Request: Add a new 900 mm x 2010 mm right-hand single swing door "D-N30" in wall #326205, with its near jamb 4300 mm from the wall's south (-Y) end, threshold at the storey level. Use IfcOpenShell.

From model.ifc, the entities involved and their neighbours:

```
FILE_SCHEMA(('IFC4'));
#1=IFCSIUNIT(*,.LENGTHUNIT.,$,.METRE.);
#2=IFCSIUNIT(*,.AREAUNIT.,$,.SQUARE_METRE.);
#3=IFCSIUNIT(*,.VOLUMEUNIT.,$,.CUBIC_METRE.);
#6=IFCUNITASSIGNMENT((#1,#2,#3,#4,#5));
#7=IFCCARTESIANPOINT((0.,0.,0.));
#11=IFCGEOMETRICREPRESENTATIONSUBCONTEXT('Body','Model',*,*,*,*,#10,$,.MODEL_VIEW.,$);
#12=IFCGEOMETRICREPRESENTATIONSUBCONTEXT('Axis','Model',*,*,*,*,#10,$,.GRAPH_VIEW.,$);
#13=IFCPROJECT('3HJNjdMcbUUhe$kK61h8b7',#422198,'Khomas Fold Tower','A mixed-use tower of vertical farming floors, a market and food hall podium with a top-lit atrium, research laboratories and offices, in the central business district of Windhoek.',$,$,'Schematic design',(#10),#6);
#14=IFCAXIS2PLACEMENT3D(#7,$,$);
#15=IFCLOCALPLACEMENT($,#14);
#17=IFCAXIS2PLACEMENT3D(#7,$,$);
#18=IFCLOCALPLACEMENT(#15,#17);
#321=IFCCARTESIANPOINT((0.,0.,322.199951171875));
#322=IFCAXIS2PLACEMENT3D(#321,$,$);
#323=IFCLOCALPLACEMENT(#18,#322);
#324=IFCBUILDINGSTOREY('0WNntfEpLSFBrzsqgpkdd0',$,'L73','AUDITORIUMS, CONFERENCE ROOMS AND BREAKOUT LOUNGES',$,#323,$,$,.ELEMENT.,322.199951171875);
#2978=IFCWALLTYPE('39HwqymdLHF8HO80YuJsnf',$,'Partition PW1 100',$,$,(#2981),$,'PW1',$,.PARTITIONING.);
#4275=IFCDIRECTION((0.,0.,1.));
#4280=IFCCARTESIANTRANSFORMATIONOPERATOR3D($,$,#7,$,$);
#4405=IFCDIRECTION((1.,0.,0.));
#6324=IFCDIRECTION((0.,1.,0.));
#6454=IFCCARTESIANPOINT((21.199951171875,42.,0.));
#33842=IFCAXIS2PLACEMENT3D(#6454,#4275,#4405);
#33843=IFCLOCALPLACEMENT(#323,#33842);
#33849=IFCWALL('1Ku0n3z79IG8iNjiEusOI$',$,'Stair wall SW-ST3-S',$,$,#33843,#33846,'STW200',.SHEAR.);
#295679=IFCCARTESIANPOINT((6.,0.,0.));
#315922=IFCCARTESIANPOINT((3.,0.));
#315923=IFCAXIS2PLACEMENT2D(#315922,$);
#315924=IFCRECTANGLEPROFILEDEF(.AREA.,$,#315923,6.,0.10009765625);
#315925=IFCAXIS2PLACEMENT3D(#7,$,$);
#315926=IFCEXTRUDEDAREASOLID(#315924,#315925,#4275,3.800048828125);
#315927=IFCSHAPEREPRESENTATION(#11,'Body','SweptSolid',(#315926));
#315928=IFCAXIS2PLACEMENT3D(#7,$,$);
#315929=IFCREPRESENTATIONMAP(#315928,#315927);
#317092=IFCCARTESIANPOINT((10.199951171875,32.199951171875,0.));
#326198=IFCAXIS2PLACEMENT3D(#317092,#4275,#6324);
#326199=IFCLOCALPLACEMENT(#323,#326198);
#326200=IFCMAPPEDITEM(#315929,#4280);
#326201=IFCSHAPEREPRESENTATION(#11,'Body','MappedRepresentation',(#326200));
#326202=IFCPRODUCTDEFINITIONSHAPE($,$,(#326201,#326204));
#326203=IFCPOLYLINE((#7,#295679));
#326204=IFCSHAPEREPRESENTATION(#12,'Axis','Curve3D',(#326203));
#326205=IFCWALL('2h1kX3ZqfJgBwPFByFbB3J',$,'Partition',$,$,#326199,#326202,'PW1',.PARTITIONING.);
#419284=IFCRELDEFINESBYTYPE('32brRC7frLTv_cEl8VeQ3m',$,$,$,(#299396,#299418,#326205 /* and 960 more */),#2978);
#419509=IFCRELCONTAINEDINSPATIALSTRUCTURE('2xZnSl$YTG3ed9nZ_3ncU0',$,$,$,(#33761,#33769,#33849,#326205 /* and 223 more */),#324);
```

```python
import numpy as np
import ifcopenshell
import ifcopenshell.api.feature
import ifcopenshell.api.geometry
import ifcopenshell.api.root
import ifcopenshell.api.spatial
import ifcopenshell.geom
import ifcopenshell.util.element
import ifcopenshell.util.placement
import ifcopenshell.util.representation
import ifcopenshell.util.shape
import ifcopenshell.util.unit

model = ifcopenshell.open("model.ifc")
unit_scale = ifcopenshell.util.unit.calculate_unit_scale(model)
settings = ifcopenshell.geom.settings()


def volume(element):
    """Net volume in cubic metres, openings subtracted."""
    shape = ifcopenshell.geom.create_shape(settings, element)
    return ifcopenshell.util.shape.get_volume(shape.geometry)


wall = model.by_id(326205)
storey = ifcopenshell.util.element.get_container(wall, ifc_class="IfcBuildingStorey")
context = ifcopenshell.util.representation.get_context(model, "Model", "Body", "MODEL_VIEW")
before = volume(wall)

width, height, from_end, sill = 0.9, 2.01, 4.3, 0.0  # metres

# The wall runs along its own X axis, and the end named is its -X end.
wall_shape = ifcopenshell.geom.create_shape(settings, wall)
x, y, z = ifcopenshell.util.shape.get_vertices(wall_shape.geometry).T
start = x.min() + from_end
face, thickness = float(y.min()), float(y.max() - y.min())
wall_matrix = ifcopenshell.util.placement.get_local_placement(wall.ObjectPlacement)
level = ifcopenshell.util.placement.get_local_placement(storey.ObjectPlacement)[2, 3]


def in_wall(x, y):
    """Placement at x, y metres in the wall's axes, at sill height."""
    matrix = wall_matrix.copy()
    matrix[:, 3] = wall_matrix @ np.array([x / unit_scale, y / unit_scale, 0.0, 1.0])
    matrix[2, 3] = level + sill / unit_scale
    return matrix


# Opening: a box that overshoots both wall faces by 50 mm.
opening = ifcopenshell.api.root.create_entity(model, ifc_class="IfcOpeningElement", predefined_type="OPENING")
box = ifcopenshell.api.geometry.add_wall_representation(
    model, context=context, length=width, height=height, thickness=thickness + 0.1
)
ifcopenshell.api.geometry.assign_representation(model, product=opening, representation=box)
ifcopenshell.api.geometry.edit_object_placement(model, product=opening, matrix=in_wall(start, face - 0.05), is_si=False)
ifcopenshell.api.feature.add_feature(model, feature=opening, element=wall)

door = ifcopenshell.api.root.create_entity(model, ifc_class="IfcDoor", name="D-N30", predefined_type="DOOR")
door.OverallWidth, door.OverallHeight = width / unit_scale, height / unit_scale
door.OperationType = "SINGLE_SWING_RIGHT"
body = ifcopenshell.api.geometry.add_door_representation(
    model,
    context=context,
    overall_width=door.OverallWidth,
    overall_height=door.OverallHeight,
    operation_type="SINGLE_SWING_RIGHT",
    lining_properties={"LiningDepth": thickness / unit_scale, "ThresholdDepth": thickness / unit_scale},
)
ifcopenshell.api.geometry.assign_representation(model, product=door, representation=body)
ifcopenshell.api.spatial.assign_container(model, products=[door], relating_structure=storey)
ifcopenshell.api.feature.add_filling(model, opening=opening, element=door)

# The lining spans the wall, so the door starts at the wall face.
ifcopenshell.api.geometry.edit_object_placement(model, product=door, matrix=in_wall(start, face), is_si=False)

after = volume(wall)

print(f"wall volume {before:.3f} -> {after:.3f} m3")

model.write("model_v2.ifc")
```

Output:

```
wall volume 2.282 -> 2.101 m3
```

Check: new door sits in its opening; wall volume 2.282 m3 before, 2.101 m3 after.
